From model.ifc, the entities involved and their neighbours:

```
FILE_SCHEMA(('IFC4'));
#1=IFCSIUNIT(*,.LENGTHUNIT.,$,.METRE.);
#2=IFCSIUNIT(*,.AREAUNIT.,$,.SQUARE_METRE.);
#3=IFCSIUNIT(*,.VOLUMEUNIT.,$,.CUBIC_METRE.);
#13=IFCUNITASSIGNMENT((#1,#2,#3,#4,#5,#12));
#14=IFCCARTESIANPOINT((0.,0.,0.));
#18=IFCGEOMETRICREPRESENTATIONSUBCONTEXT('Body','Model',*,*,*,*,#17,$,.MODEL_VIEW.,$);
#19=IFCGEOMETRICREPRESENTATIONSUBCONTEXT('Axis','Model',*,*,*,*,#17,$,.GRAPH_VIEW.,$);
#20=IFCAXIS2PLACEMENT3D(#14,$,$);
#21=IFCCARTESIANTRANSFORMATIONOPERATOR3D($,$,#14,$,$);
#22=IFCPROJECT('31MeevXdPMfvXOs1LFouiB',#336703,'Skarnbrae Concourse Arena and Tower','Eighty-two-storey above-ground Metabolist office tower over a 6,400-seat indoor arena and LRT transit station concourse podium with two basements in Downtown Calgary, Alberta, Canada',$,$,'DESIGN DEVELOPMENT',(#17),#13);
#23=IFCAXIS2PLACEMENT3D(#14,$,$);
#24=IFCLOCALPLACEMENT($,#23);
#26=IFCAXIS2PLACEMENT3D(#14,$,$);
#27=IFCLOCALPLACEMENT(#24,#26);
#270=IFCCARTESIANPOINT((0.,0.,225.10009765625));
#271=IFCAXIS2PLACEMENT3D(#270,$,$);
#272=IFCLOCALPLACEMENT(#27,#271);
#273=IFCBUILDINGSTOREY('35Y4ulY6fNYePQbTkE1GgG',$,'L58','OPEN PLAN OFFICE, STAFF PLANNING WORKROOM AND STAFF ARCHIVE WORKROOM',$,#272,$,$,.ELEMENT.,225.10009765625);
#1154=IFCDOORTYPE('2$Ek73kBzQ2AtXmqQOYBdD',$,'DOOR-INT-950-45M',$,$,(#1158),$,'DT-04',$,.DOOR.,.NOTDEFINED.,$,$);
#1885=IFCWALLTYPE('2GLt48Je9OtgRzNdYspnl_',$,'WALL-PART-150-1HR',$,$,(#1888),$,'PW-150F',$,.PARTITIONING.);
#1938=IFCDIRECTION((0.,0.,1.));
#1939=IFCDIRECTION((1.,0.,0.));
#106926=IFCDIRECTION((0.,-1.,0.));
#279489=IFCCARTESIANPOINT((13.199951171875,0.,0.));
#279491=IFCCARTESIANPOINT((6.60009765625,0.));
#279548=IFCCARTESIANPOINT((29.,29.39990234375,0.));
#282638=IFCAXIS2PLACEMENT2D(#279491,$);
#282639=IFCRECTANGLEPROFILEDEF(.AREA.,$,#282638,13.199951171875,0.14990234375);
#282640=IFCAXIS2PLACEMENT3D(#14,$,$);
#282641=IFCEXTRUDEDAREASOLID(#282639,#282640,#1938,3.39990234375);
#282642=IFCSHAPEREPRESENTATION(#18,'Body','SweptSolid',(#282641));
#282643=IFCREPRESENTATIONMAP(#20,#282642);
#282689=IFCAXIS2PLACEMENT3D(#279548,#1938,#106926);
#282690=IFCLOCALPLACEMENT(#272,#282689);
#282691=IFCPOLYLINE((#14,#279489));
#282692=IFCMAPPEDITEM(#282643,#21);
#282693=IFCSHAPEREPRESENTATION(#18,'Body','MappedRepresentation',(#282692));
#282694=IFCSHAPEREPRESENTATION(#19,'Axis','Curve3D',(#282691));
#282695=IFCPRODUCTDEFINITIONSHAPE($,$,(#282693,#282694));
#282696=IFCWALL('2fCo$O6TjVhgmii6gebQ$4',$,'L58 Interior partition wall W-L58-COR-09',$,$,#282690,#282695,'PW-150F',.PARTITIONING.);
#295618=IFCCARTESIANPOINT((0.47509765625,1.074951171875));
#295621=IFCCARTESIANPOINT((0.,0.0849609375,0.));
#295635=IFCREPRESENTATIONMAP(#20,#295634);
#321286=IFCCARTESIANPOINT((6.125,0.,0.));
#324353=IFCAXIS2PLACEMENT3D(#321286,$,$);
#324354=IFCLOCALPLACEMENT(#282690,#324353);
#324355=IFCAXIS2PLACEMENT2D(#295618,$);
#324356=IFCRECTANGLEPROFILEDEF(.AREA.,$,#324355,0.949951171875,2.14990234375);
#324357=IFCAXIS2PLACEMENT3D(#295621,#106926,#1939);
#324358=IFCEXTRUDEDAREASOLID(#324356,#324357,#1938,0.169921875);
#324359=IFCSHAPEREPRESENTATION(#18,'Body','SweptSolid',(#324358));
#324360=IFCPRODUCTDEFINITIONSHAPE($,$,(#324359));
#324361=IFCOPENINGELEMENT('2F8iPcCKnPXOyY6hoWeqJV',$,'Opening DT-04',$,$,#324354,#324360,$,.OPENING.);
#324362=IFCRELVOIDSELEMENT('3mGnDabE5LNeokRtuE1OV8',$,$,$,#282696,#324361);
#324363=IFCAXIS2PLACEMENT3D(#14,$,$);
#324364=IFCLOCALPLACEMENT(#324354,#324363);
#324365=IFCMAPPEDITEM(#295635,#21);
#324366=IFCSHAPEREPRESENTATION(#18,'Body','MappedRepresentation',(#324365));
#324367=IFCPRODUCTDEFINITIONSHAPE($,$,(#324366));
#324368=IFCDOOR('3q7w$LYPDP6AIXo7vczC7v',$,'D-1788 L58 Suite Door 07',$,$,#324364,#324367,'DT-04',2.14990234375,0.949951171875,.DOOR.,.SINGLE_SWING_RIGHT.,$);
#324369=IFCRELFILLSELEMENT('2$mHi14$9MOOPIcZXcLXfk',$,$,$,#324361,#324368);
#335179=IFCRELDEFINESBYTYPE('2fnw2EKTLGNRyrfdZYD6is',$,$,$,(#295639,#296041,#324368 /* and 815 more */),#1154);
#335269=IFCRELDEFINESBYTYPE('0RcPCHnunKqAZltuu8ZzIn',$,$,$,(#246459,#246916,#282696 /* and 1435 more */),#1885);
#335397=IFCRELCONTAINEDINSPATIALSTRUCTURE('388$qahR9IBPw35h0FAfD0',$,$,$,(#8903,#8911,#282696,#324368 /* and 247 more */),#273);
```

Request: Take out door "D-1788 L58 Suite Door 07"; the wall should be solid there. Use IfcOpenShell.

```python
import ifcopenshell
import ifcopenshell.api.feature
import ifcopenshell.api.root
import ifcopenshell.geom
import ifcopenshell.util.shape

model = ifcopenshell.open("model.ifc")
settings = ifcopenshell.geom.settings()


def volume(element):
    """Net volume in cubic metres, openings subtracted."""
    shape = ifcopenshell.geom.create_shape(settings, element)
    return ifcopenshell.util.shape.get_volume(shape.geometry)


door = model.by_guid("3q7w$LYPDP6AIXo7vczC7v")
opening = door.FillsVoids[0].RelatingOpeningElement
wall = opening.VoidsElements[0].RelatingBuildingElement
before = volume(wall)

ifcopenshell.api.root.remove_product(model, product=door)
ifcopenshell.api.feature.remove_feature(model, feature=opening)

after = volume(wall)

print(f"wall volume {before:.3f} -> {after:.3f} m3")

model.write("model-out.ifc")
```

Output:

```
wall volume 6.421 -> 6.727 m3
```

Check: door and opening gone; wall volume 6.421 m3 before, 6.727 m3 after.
